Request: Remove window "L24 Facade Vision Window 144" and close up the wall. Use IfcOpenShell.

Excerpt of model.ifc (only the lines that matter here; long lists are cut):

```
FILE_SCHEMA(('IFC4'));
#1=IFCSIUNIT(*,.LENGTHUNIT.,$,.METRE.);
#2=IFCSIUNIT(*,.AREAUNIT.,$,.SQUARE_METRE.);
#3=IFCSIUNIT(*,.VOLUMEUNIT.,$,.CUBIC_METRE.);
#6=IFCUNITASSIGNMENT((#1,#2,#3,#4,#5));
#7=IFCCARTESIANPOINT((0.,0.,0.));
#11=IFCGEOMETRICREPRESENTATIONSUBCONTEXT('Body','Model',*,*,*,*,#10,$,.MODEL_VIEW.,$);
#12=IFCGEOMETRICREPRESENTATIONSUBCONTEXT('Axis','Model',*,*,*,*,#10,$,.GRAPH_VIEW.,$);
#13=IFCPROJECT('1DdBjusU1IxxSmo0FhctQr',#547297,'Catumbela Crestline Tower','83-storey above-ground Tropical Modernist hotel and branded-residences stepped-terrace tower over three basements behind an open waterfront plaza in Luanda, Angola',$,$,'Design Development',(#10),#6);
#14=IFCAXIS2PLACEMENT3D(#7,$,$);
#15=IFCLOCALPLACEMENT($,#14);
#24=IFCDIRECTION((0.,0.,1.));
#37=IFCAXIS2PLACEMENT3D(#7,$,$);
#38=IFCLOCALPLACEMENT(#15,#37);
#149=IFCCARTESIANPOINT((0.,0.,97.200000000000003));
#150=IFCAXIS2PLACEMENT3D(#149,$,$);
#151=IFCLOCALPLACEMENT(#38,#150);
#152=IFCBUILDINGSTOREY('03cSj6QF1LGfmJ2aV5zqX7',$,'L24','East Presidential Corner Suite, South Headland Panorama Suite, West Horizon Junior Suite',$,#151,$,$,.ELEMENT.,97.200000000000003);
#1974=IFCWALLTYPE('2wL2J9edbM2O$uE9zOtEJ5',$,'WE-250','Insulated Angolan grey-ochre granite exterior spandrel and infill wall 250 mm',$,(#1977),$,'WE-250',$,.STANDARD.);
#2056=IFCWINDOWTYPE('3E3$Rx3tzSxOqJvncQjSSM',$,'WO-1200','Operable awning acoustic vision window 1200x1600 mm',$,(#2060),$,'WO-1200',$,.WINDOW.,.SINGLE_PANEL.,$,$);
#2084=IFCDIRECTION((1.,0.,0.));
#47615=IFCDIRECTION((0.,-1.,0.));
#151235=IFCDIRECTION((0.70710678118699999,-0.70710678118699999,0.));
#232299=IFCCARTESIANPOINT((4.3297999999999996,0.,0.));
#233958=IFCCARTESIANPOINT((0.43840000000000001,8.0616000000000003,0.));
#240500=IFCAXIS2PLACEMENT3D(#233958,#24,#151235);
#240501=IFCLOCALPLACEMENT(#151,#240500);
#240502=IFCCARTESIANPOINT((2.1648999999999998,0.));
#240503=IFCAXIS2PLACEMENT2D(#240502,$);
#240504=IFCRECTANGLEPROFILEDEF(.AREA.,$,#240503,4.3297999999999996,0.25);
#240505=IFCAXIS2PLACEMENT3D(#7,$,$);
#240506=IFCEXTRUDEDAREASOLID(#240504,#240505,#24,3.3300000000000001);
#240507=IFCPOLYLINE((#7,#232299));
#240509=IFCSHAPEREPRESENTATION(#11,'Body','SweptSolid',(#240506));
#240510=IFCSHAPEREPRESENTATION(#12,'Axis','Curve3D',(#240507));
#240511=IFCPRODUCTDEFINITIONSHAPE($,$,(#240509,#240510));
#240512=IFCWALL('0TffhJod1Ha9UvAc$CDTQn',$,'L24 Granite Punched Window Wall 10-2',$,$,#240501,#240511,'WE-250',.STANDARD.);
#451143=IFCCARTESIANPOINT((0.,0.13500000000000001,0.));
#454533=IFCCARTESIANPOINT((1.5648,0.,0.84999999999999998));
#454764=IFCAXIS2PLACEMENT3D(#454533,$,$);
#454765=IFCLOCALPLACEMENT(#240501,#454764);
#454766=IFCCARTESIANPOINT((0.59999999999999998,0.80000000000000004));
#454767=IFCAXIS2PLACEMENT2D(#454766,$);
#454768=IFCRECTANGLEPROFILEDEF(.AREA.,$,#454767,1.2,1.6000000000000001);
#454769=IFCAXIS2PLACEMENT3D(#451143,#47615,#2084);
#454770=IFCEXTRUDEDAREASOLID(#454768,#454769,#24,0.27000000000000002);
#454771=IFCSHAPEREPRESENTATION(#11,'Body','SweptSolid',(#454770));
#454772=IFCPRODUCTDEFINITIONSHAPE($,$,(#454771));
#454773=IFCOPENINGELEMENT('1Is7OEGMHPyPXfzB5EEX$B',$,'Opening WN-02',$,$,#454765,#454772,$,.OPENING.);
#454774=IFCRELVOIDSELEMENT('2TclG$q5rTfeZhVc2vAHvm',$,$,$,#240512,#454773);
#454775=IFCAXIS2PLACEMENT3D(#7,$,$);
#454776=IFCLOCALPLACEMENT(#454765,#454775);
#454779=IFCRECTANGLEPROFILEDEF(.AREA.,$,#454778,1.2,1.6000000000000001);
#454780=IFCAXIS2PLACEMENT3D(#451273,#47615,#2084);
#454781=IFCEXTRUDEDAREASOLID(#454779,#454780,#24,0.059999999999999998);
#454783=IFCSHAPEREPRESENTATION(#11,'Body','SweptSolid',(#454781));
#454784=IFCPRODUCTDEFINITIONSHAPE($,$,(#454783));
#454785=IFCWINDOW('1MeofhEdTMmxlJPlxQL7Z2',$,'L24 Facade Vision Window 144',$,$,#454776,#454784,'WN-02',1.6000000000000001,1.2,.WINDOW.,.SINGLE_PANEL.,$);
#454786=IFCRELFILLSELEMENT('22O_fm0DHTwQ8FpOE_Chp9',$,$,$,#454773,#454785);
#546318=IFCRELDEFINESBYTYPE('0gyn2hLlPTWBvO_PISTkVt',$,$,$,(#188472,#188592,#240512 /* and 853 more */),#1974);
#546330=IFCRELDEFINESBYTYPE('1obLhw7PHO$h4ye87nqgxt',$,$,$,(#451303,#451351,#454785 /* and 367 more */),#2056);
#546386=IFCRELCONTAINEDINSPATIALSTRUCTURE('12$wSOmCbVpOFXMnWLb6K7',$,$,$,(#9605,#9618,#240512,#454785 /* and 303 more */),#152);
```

```python
import ifcopenshell
import ifcopenshell.api.feature
import ifcopenshell.api.root
import ifcopenshell.geom
import ifcopenshell.util.shape

model = ifcopenshell.open("model.ifc")
settings = ifcopenshell.geom.settings()


def volume(element):
    """Net volume in cubic metres, openings subtracted."""
    shape = ifcopenshell.geom.create_shape(settings, element)
    return ifcopenshell.util.shape.get_volume(shape.geometry)


window = model.by_guid("1MeofhEdTMmxlJPlxQL7Z2")
opening = window.FillsVoids[0].RelatingOpeningElement
wall = opening.VoidsElements[0].RelatingBuildingElement
before = volume(wall)

ifcopenshell.api.root.remove_product(model, product=window)
ifcopenshell.api.feature.remove_feature(model, feature=opening)

after = volume(wall)

print(f"wall volume {before:.3f} -> {after:.3f} m3")

model.write("model_updated.ifc")
```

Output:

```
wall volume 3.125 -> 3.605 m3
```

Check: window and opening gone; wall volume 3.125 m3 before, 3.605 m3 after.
